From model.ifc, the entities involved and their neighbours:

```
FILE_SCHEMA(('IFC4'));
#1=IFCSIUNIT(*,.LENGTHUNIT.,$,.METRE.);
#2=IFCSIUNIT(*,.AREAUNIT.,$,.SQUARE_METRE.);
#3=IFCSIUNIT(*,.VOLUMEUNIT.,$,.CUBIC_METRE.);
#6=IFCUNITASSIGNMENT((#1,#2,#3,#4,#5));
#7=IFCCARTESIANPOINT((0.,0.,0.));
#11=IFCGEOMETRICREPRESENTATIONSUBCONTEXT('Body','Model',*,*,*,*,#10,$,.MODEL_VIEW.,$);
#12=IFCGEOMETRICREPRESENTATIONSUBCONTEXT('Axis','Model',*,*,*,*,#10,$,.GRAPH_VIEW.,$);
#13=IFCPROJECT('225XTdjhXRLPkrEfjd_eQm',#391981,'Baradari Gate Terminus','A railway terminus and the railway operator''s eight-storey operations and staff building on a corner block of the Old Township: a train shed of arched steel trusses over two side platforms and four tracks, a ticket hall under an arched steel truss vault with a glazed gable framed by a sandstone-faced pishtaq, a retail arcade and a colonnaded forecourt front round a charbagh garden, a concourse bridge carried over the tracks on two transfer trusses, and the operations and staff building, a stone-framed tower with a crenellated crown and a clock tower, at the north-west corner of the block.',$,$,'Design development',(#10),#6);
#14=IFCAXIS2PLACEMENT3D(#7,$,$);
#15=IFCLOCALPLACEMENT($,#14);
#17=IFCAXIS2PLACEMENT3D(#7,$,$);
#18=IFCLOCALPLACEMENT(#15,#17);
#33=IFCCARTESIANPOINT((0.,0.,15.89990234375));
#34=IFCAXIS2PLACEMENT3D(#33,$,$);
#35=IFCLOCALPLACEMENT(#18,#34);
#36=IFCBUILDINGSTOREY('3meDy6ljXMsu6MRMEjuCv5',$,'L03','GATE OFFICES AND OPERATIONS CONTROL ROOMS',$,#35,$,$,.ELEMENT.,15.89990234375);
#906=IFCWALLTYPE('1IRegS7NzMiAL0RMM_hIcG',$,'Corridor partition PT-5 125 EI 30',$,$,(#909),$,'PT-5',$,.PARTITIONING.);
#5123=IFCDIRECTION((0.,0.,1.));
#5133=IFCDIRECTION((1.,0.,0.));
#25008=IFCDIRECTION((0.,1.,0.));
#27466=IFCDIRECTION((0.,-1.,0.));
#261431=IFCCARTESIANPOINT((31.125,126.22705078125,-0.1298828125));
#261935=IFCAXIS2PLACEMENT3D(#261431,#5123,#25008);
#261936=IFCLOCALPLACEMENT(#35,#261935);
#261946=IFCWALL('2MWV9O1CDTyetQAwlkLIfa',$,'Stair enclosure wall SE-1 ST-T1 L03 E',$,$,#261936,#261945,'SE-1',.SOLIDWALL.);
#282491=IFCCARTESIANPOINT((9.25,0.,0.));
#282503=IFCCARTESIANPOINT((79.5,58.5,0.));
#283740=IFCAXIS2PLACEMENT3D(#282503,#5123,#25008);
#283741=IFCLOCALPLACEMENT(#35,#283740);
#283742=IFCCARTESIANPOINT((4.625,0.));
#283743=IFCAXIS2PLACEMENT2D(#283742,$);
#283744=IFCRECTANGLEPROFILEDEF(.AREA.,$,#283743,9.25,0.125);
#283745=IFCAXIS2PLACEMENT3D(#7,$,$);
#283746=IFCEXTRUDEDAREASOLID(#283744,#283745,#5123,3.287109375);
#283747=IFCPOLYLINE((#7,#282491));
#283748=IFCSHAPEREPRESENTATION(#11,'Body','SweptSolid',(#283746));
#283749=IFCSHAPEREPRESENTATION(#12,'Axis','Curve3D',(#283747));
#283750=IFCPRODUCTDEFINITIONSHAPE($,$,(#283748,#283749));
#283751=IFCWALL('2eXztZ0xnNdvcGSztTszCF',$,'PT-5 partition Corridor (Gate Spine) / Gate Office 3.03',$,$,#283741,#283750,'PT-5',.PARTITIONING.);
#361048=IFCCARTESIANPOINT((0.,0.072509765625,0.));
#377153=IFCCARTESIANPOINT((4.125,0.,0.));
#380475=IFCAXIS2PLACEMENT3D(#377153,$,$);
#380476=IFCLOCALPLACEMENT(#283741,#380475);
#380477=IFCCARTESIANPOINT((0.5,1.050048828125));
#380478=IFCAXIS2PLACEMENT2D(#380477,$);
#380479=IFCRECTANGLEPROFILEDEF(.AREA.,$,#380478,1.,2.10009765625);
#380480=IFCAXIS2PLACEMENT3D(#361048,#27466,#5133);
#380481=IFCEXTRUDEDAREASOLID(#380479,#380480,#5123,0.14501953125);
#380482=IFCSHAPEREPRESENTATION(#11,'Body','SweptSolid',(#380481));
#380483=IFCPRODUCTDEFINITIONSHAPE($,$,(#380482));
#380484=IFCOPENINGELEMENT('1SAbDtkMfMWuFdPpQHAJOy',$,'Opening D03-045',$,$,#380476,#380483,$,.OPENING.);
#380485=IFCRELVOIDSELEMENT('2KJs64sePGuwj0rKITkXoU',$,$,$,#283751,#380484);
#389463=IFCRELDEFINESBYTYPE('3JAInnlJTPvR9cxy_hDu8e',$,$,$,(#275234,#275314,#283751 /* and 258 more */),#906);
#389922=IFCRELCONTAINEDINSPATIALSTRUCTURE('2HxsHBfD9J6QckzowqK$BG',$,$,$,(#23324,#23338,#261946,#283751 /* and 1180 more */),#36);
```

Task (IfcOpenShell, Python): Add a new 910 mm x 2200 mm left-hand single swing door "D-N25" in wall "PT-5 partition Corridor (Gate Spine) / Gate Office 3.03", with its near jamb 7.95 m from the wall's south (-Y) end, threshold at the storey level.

```python
import numpy as np
import ifcopenshell
import ifcopenshell.api.feature
import ifcopenshell.api.geometry
import ifcopenshell.api.root
import ifcopenshell.api.spatial
import ifcopenshell.geom
import ifcopenshell.util.element
import ifcopenshell.util.placement
import ifcopenshell.util.representation
import ifcopenshell.util.shape
import ifcopenshell.util.unit

model = ifcopenshell.open("model.ifc")
unit_scale = ifcopenshell.util.unit.calculate_unit_scale(model)
settings = ifcopenshell.geom.settings()


def volume(element):
    """Net volume in cubic metres, openings subtracted."""
    shape = ifcopenshell.geom.create_shape(settings, element)
    return ifcopenshell.util.shape.get_volume(shape.geometry)


wall = model.by_id(283751)
storey = ifcopenshell.util.element.get_container(wall, ifc_class="IfcBuildingStorey")
context = ifcopenshell.util.representation.get_context(model, "Model", "Body", "MODEL_VIEW")
before = volume(wall)

width, height, from_end, sill = 0.91, 2.2, 7.95, 0.0  # metres

# The wall runs along its own X axis, and the end named is its -X end.
wall_shape = ifcopenshell.geom.create_shape(settings, wall)
x, y, z = ifcopenshell.util.shape.get_vertices(wall_shape.geometry).T
start = x.min() + from_end
face, thickness = float(y.min()), float(y.max() - y.min())
wall_matrix = ifcopenshell.util.placement.get_local_placement(wall.ObjectPlacement)
level = ifcopenshell.util.placement.get_local_placement(storey.ObjectPlacement)[2, 3]


def in_wall(x, y):
    """Placement at x, y metres in the wall's axes, at sill height."""
    matrix = wall_matrix.copy()
    matrix[:, 3] = wall_matrix @ np.array([x / unit_scale, y / unit_scale, 0.0, 1.0])
    matrix[2, 3] = level + sill / unit_scale
    return matrix


# Opening: a box that overshoots both wall faces by 50 mm.
opening = ifcopenshell.api.root.create_entity(model, ifc_class="IfcOpeningElement", predefined_type="OPENING")
box = ifcopenshell.api.geometry.add_wall_representation(
    model, context=context, length=width, height=height, thickness=thickness + 0.1
)
ifcopenshell.api.geometry.assign_representation(model, product=opening, representation=box)
ifcopenshell.api.geometry.edit_object_placement(model, product=opening, matrix=in_wall(start, face - 0.05), is_si=False)
ifcopenshell.api.feature.add_feature(model, feature=opening, element=wall)

door = ifcopenshell.api.root.create_entity(model, ifc_class="IfcDoor", name="D-N25", predefined_type="DOOR")
door.OverallWidth, door.OverallHeight = width / unit_scale, height / unit_scale
door.OperationType = "SINGLE_SWING_LEFT"
body = ifcopenshell.api.geometry.add_door_representation(
    model,
    context=context,
    overall_width=door.OverallWidth,
    overall_height=door.OverallHeight,
    operation_type="SINGLE_SWING_LEFT",
    lining_properties={"LiningDepth": thickness / unit_scale, "ThresholdDepth": thickness / unit_scale},
)
ifcopenshell.api.geometry.assign_representation(model, product=door, representation=body)
ifcopenshell.api.spatial.assign_container(model, products=[door], relating_structure=storey)
ifcopenshell.api.feature.add_filling(model, opening=opening, element=door)

# The lining spans the wall, so the door starts at the wall face.
ifcopenshell.api.geometry.edit_object_placement(model, product=door, matrix=in_wall(start, face), is_si=False)

after = volume(wall)

print(f"wall volume {before:.3f} -> {after:.3f} m3")

model.write("model_rev.ifc")
```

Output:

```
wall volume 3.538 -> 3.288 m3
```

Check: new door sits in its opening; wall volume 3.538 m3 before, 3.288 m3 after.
